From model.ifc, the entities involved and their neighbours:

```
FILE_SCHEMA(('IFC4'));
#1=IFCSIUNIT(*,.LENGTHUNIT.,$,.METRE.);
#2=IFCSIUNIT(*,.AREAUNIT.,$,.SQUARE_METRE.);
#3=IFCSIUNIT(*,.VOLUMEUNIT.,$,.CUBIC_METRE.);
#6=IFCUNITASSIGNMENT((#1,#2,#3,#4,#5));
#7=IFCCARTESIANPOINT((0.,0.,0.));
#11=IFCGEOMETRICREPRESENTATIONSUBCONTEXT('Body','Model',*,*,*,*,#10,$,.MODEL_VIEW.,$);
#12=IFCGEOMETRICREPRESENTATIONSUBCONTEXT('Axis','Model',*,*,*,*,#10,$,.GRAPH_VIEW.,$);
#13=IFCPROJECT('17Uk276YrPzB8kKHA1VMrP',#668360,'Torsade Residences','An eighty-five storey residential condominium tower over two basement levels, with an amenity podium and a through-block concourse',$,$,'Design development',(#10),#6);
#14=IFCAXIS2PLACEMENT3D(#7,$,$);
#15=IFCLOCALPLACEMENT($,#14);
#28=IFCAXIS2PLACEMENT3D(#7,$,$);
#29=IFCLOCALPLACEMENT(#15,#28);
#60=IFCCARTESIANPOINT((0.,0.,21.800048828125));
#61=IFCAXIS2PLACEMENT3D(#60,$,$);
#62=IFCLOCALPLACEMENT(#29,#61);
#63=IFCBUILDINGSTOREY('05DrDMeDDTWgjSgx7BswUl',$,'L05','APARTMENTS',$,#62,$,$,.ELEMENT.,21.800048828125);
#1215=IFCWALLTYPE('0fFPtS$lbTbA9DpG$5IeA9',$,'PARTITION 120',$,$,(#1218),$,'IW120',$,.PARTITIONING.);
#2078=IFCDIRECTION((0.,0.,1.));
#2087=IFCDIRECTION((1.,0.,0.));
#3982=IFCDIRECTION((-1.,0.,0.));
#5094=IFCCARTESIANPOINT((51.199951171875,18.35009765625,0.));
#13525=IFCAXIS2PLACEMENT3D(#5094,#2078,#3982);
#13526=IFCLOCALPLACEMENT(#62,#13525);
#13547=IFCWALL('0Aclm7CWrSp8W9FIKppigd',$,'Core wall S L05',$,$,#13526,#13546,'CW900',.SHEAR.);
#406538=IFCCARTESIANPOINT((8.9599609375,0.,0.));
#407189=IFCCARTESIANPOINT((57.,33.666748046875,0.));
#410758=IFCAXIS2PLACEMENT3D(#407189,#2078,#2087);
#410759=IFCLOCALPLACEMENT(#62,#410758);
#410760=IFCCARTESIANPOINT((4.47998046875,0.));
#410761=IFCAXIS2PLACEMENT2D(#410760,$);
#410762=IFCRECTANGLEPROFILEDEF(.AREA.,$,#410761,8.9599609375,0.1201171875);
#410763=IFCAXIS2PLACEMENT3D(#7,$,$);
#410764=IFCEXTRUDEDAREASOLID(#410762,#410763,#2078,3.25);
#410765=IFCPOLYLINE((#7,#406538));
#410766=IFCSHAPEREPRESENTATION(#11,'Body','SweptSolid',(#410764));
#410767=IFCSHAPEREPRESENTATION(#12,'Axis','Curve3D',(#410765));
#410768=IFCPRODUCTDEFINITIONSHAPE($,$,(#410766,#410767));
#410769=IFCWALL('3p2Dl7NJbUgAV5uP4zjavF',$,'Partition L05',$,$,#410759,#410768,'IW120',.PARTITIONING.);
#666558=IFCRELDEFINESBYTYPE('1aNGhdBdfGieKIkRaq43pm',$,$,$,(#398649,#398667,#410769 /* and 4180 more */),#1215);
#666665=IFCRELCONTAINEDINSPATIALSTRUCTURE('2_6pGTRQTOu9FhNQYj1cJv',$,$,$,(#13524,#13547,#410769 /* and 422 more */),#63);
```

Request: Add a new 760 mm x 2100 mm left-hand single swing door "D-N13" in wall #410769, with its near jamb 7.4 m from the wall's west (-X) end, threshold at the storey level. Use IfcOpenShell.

```python
import numpy as np
import ifcopenshell
import ifcopenshell.api.feature
import ifcopenshell.api.geometry
import ifcopenshell.api.root
import ifcopenshell.api.spatial
import ifcopenshell.geom
import ifcopenshell.util.element
import ifcopenshell.util.placement
import ifcopenshell.util.representation
import ifcopenshell.util.shape
import ifcopenshell.util.unit

model = ifcopenshell.open("model.ifc")
unit_scale = ifcopenshell.util.unit.calculate_unit_scale(model)
settings = ifcopenshell.geom.settings()


def volume(element):
    """Net volume in cubic metres, openings subtracted."""
    shape = ifcopenshell.geom.create_shape(settings, element)
    return ifcopenshell.util.shape.get_volume(shape.geometry)


wall = model.by_guid("3p2Dl7NJbUgAV5uP4zjavF")
storey = ifcopenshell.util.element.get_container(wall, ifc_class="IfcBuildingStorey")
context = ifcopenshell.util.representation.get_context(model, "Model", "Body", "MODEL_VIEW")
before = volume(wall)

width, height, from_end, sill = 0.76, 2.1, 7.4, 0.0  # metres

# The wall runs along its own X axis, and the end named is its -X end.
wall_shape = ifcopenshell.geom.create_shape(settings, wall)
x, y, z = ifcopenshell.util.shape.get_vertices(wall_shape.geometry).T
start = x.min() + from_end
face, thickness = float(y.min()), float(y.max() - y.min())
wall_matrix = ifcopenshell.util.placement.get_local_placement(wall.ObjectPlacement)
level = ifcopenshell.util.placement.get_local_placement(storey.ObjectPlacement)[2, 3]


def in_wall(x, y):
    """Placement at x, y metres in the wall's axes, at sill height."""
    matrix = wall_matrix.copy()
    matrix[:, 3] = wall_matrix @ np.array([x / unit_scale, y / unit_scale, 0.0, 1.0])
    matrix[2, 3] = level + sill / unit_scale
    return matrix


# Opening: a box that overshoots both wall faces by 50 mm.
opening = ifcopenshell.api.root.create_entity(model, ifc_class="IfcOpeningElement", predefined_type="OPENING")
box = ifcopenshell.api.geometry.add_wall_representation(
    model, context=context, length=width, height=height, thickness=thickness + 0.1
)
ifcopenshell.api.geometry.assign_representation(model, product=opening, representation=box)
ifcopenshell.api.geometry.edit_object_placement(model, product=opening, matrix=in_wall(start, face - 0.05), is_si=False)
ifcopenshell.api.feature.add_feature(model, feature=opening, element=wall)

door = ifcopenshell.api.root.create_entity(model, ifc_class="IfcDoor", name="D-N13", predefined_type="DOOR")
door.OverallWidth, door.OverallHeight = width / unit_scale, height / unit_scale
door.OperationType = "SINGLE_SWING_LEFT"
body = ifcopenshell.api.geometry.add_door_representation(
    model,
    context=context,
    overall_width=door.OverallWidth,
    overall_height=door.OverallHeight,
    operation_type="SINGLE_SWING_LEFT",
    lining_properties={"LiningDepth": thickness / unit_scale, "ThresholdDepth": thickness / unit_scale},
)
ifcopenshell.api.geometry.assign_representation(model, product=door, representation=body)
ifcopenshell.api.spatial.assign_container(model, products=[door], relating_structure=storey)
ifcopenshell.api.feature.add_filling(model, opening=opening, element=door)

# The lining spans the wall, so the door starts at the wall face.
ifcopenshell.api.geometry.edit_object_placement(model, product=door, matrix=in_wall(start, face), is_si=False)

after = volume(wall)

print(f"wall volume {before:.3f} -> {after:.3f} m3")

model.write("model-out.ifc")
```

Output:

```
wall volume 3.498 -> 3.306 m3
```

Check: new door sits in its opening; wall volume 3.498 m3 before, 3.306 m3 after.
